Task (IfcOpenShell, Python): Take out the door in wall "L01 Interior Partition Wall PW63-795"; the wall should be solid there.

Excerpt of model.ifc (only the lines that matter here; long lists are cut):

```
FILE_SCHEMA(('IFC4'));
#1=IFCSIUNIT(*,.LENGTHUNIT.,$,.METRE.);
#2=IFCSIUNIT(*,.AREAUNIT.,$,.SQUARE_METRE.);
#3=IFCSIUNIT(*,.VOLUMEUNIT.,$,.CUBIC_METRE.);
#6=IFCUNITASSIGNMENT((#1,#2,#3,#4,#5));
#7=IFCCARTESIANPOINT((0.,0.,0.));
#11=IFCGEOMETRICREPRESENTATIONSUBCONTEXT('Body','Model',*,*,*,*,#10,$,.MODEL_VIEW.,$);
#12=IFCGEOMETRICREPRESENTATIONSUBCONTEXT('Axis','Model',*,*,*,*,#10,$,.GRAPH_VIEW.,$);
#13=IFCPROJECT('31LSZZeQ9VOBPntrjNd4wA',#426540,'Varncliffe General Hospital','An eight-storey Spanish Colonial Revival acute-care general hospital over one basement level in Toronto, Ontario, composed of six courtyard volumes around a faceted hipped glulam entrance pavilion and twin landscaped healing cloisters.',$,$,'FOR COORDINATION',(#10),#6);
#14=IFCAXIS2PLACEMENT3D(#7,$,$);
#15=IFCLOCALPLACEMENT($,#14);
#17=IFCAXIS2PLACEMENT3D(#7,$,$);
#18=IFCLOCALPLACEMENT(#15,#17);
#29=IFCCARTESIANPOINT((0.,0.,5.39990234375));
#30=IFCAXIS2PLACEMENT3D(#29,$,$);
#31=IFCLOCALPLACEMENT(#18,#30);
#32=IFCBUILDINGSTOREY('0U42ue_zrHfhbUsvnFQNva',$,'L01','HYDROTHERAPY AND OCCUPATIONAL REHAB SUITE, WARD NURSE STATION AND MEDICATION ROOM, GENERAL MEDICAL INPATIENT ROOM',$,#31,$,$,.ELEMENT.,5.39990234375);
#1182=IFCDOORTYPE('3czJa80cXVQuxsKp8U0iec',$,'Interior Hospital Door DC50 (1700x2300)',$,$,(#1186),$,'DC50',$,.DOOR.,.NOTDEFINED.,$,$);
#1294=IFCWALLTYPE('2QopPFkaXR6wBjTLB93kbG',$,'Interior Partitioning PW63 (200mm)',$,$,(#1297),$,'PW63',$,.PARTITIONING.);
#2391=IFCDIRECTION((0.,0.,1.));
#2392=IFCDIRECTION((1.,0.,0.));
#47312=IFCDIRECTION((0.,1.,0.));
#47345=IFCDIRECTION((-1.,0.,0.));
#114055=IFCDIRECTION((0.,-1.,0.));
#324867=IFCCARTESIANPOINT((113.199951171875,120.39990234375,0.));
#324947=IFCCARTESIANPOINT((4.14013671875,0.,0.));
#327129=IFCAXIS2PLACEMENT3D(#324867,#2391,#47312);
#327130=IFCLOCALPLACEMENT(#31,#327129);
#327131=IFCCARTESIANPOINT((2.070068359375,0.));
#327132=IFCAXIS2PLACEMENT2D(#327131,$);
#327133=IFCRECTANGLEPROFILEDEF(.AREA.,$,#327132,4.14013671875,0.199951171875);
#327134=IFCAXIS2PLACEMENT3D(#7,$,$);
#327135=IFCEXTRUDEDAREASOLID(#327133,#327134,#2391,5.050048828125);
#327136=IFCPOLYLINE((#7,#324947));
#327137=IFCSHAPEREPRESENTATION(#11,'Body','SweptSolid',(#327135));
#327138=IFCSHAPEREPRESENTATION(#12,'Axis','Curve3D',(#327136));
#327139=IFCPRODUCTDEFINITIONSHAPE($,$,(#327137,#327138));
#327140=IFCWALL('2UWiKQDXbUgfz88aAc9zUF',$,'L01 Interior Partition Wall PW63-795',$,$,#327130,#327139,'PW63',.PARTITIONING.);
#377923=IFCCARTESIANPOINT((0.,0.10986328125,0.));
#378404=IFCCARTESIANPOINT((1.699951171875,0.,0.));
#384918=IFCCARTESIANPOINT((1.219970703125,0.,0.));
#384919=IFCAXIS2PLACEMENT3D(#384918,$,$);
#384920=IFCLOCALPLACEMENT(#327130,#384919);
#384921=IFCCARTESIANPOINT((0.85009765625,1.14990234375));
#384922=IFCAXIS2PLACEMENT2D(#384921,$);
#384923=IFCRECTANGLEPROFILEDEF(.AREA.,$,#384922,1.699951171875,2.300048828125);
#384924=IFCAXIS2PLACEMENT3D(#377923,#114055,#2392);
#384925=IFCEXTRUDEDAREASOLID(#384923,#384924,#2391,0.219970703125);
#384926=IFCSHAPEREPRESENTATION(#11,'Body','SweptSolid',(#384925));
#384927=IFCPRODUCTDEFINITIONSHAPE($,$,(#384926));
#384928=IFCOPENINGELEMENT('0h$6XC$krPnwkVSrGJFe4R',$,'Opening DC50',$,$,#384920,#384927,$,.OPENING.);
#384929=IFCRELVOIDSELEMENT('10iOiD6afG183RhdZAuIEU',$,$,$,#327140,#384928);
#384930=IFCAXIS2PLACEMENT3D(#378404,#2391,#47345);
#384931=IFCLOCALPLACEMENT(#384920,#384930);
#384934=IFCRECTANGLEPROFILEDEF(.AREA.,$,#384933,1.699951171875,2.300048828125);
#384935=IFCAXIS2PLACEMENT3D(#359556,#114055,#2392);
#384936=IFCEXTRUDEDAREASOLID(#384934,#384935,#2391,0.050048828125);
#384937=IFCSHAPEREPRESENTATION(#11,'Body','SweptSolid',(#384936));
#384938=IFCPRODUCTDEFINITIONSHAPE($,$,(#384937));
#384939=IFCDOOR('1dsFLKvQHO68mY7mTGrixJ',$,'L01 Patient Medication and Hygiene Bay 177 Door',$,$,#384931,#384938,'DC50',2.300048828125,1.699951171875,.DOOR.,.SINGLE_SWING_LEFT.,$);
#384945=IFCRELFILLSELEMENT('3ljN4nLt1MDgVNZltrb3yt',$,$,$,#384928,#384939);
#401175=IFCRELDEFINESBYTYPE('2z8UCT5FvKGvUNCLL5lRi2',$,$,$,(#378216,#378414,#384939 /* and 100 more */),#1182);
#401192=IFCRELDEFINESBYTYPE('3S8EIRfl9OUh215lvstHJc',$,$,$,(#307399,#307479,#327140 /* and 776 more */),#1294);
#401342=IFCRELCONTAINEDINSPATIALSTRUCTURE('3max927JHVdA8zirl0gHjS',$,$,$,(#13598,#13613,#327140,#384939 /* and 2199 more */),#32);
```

```python
import ifcopenshell
import ifcopenshell.api.feature
import ifcopenshell.api.root
import ifcopenshell.geom
import ifcopenshell.util.shape

model = ifcopenshell.open("model.ifc")
settings = ifcopenshell.geom.settings()


def volume(element):
    """Net volume in cubic metres, openings subtracted."""
    shape = ifcopenshell.geom.create_shape(settings, element)
    return ifcopenshell.util.shape.get_volume(shape.geometry)


door = model.by_guid("1dsFLKvQHO68mY7mTGrixJ")
opening = door.FillsVoids[0].RelatingOpeningElement
wall = opening.VoidsElements[0].RelatingBuildingElement
before = volume(wall)

ifcopenshell.api.root.remove_product(model, product=door)
ifcopenshell.api.feature.remove_feature(model, feature=opening)

after = volume(wall)

print(f"wall volume {before:.3f} -> {after:.3f} m3")

model.write("model-out.ifc")
```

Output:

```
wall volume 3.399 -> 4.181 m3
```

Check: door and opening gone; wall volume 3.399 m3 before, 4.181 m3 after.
